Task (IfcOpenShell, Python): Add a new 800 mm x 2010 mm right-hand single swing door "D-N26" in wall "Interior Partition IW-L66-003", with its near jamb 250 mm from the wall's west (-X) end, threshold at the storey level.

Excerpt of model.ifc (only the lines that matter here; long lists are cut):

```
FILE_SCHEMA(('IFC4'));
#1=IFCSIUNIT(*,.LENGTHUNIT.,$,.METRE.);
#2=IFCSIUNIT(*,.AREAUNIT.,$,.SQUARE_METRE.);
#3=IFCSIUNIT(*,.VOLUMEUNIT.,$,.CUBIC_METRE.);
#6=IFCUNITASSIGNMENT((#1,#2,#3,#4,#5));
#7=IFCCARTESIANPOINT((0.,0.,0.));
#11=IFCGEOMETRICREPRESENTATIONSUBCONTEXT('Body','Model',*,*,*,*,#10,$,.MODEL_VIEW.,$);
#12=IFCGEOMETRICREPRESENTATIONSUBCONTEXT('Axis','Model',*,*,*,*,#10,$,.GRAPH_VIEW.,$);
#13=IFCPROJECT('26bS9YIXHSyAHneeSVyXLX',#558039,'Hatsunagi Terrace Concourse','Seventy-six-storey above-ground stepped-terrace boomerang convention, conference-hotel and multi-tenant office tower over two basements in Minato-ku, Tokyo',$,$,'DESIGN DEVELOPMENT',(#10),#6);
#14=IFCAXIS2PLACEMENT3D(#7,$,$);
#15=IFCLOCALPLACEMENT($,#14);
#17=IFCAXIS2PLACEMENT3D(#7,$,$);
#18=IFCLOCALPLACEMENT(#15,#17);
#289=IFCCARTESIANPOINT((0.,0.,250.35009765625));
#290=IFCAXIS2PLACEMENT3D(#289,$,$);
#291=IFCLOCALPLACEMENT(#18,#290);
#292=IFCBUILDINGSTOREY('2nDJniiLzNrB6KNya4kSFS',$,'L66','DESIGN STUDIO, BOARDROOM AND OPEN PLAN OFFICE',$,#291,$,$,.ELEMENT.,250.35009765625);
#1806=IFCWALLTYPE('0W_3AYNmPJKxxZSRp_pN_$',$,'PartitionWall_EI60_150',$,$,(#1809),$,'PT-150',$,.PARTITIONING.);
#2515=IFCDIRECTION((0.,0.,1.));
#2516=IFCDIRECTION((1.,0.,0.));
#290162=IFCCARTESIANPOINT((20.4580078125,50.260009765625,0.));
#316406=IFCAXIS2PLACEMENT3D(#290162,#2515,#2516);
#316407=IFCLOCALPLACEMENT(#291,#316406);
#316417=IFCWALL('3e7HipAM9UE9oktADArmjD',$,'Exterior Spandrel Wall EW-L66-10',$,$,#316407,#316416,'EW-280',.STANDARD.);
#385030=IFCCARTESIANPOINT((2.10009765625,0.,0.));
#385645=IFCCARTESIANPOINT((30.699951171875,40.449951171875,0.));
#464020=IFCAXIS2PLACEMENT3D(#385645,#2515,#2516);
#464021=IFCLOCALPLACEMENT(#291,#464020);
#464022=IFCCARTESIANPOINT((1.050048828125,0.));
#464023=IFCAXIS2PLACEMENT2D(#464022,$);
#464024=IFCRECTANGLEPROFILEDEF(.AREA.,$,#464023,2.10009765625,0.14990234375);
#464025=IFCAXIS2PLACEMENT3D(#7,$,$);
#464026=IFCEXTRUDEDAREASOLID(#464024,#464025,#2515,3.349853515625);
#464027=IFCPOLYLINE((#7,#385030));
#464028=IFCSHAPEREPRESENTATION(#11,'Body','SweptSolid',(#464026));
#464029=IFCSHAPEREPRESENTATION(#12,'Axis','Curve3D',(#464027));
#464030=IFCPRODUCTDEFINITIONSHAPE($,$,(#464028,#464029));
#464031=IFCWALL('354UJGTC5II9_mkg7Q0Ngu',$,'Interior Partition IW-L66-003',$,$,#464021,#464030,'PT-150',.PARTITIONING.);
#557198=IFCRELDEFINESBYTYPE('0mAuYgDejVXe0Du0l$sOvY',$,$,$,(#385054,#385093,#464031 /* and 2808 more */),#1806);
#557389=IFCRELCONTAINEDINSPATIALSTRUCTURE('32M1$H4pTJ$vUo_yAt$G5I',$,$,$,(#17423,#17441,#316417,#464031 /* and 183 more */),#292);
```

```python
import numpy as np
import ifcopenshell
import ifcopenshell.api.feature
import ifcopenshell.api.geometry
import ifcopenshell.api.root
import ifcopenshell.api.spatial
import ifcopenshell.geom
import ifcopenshell.util.element
import ifcopenshell.util.placement
import ifcopenshell.util.representation
import ifcopenshell.util.shape
import ifcopenshell.util.unit

model = ifcopenshell.open("model.ifc")
unit_scale = ifcopenshell.util.unit.calculate_unit_scale(model)
settings = ifcopenshell.geom.settings()


def volume(element):
    """Net volume in cubic metres, openings subtracted."""
    shape = ifcopenshell.geom.create_shape(settings, element)
    return ifcopenshell.util.shape.get_volume(shape.geometry)


wall = model.by_guid("354UJGTC5II9_mkg7Q0Ngu")
storey = ifcopenshell.util.element.get_container(wall, ifc_class="IfcBuildingStorey")
context = ifcopenshell.util.representation.get_context(model, "Model", "Body", "MODEL_VIEW")
before = volume(wall)

width, height, from_end, sill = 0.8, 2.01, 0.25, 0.0  # metres

# The wall runs along its own X axis, and the end named is its -X end.
wall_shape = ifcopenshell.geom.create_shape(settings, wall)
x, y, z = ifcopenshell.util.shape.get_vertices(wall_shape.geometry).T
start = x.min() + from_end
face, thickness = float(y.min()), float(y.max() - y.min())
wall_matrix = ifcopenshell.util.placement.get_local_placement(wall.ObjectPlacement)
level = ifcopenshell.util.placement.get_local_placement(storey.ObjectPlacement)[2, 3]


def in_wall(x, y):
    """Placement at x, y metres in the wall's axes, at sill height."""
    matrix = wall_matrix.copy()
    matrix[:, 3] = wall_matrix @ np.array([x / unit_scale, y / unit_scale, 0.0, 1.0])
    matrix[2, 3] = level + sill / unit_scale
    return matrix


# Opening: a box that overshoots both wall faces by 50 mm.
opening = ifcopenshell.api.root.create_entity(model, ifc_class="IfcOpeningElement", predefined_type="OPENING")
box = ifcopenshell.api.geometry.add_wall_representation(
    model, context=context, length=width, height=height, thickness=thickness + 0.1
)
ifcopenshell.api.geometry.assign_representation(model, product=opening, representation=box)
ifcopenshell.api.geometry.edit_object_placement(model, product=opening, matrix=in_wall(start, face - 0.05), is_si=False)
ifcopenshell.api.feature.add_feature(model, feature=opening, element=wall)

door = ifcopenshell.api.root.create_entity(model, ifc_class="IfcDoor", name="D-N26", predefined_type="DOOR")
door.OverallWidth, door.OverallHeight = width / unit_scale, height / unit_scale
door.OperationType = "SINGLE_SWING_RIGHT"
body = ifcopenshell.api.geometry.add_door_representation(
    model,
    context=context,
    overall_width=door.OverallWidth,
    overall_height=door.OverallHeight,
    operation_type="SINGLE_SWING_RIGHT",
    lining_properties={"LiningDepth": thickness / unit_scale, "ThresholdDepth": thickness / unit_scale},
)
ifcopenshell.api.geometry.assign_representation(model, product=door, representation=body)
ifcopenshell.api.spatial.assign_container(model, products=[door], relating_structure=storey)
ifcopenshell.api.feature.add_filling(model, opening=opening, element=door)

# The lining spans the wall, so the door starts at the wall face.
ifcopenshell.api.geometry.edit_object_placement(model, product=door, matrix=in_wall(start, face), is_si=False)

after = volume(wall)

print(f"wall volume {before:.3f} -> {after:.3f} m3")

model.write("model_edited.ifc")
```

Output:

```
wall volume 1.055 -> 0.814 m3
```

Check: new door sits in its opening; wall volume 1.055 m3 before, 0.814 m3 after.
